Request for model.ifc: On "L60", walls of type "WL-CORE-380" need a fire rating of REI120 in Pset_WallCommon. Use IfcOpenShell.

First a look at what the model holds.

```python
import ifcopenshell
import ifcopenshell.util.element

model = ifcopenshell.open("model.ifc")
print(model.schema)
storey = next(s for s in model.by_type("IfcBuildingStorey") if s.Name == "L60")
walls = [e for e in ifcopenshell.util.element.get_decomposition(storey) if e.is_a("IfcWall")]
seen = {}
for e in walls:
    element_type = ifcopenshell.util.element.get_type(e)
    key = (element_type.Name if element_type != e and element_type else None, ifcopenshell.util.element.get_pset(e, "Pset_WallCommon", "FireRating"))
    seen[key] = seen.get(key, 0) + 1
for (name, value), count in sorted(seen.items(), key=str):
    print(count, "x", name, "|", value)
```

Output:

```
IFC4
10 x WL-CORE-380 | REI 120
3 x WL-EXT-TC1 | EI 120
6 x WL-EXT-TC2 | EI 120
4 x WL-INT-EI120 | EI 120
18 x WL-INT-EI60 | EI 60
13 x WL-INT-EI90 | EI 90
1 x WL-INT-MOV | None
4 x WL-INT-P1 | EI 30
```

```python
import ifcopenshell
import ifcopenshell.api.pset
import ifcopenshell.util.element

model = ifcopenshell.open("model.ifc")

storey = next(s for s in model.by_type("IfcBuildingStorey") if s.Name == "L60")
walls = [e for e in ifcopenshell.util.element.get_decomposition(storey) if e.is_a("IfcWall")]

count = 0
for e in walls:
    element_type = ifcopenshell.util.element.get_type(e)
    if element_type in (None, e) or element_type.Name != "WL-CORE-380":
        continue
    found = ifcopenshell.util.element.get_pset(e, "Pset_WallCommon", should_inherit=False)
    if found:
        pset = model.by_id(found["id"])
        if len(ifcopenshell.util.element.get_elements_by_pset(pset)) > 1:
            pset = ifcopenshell.api.pset.unshare_pset(model, products=[e], pset=pset)[0]
    else:
        pset = ifcopenshell.api.pset.add_pset(model, product=e, name="Pset_WallCommon")
    ifcopenshell.api.pset.edit_pset(model, pset=pset, properties={"FireRating": "REI120"})
    count += 1

print(count, "walls updated")

model.write("model_updated.ifc")
```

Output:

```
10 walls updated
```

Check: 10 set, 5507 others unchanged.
